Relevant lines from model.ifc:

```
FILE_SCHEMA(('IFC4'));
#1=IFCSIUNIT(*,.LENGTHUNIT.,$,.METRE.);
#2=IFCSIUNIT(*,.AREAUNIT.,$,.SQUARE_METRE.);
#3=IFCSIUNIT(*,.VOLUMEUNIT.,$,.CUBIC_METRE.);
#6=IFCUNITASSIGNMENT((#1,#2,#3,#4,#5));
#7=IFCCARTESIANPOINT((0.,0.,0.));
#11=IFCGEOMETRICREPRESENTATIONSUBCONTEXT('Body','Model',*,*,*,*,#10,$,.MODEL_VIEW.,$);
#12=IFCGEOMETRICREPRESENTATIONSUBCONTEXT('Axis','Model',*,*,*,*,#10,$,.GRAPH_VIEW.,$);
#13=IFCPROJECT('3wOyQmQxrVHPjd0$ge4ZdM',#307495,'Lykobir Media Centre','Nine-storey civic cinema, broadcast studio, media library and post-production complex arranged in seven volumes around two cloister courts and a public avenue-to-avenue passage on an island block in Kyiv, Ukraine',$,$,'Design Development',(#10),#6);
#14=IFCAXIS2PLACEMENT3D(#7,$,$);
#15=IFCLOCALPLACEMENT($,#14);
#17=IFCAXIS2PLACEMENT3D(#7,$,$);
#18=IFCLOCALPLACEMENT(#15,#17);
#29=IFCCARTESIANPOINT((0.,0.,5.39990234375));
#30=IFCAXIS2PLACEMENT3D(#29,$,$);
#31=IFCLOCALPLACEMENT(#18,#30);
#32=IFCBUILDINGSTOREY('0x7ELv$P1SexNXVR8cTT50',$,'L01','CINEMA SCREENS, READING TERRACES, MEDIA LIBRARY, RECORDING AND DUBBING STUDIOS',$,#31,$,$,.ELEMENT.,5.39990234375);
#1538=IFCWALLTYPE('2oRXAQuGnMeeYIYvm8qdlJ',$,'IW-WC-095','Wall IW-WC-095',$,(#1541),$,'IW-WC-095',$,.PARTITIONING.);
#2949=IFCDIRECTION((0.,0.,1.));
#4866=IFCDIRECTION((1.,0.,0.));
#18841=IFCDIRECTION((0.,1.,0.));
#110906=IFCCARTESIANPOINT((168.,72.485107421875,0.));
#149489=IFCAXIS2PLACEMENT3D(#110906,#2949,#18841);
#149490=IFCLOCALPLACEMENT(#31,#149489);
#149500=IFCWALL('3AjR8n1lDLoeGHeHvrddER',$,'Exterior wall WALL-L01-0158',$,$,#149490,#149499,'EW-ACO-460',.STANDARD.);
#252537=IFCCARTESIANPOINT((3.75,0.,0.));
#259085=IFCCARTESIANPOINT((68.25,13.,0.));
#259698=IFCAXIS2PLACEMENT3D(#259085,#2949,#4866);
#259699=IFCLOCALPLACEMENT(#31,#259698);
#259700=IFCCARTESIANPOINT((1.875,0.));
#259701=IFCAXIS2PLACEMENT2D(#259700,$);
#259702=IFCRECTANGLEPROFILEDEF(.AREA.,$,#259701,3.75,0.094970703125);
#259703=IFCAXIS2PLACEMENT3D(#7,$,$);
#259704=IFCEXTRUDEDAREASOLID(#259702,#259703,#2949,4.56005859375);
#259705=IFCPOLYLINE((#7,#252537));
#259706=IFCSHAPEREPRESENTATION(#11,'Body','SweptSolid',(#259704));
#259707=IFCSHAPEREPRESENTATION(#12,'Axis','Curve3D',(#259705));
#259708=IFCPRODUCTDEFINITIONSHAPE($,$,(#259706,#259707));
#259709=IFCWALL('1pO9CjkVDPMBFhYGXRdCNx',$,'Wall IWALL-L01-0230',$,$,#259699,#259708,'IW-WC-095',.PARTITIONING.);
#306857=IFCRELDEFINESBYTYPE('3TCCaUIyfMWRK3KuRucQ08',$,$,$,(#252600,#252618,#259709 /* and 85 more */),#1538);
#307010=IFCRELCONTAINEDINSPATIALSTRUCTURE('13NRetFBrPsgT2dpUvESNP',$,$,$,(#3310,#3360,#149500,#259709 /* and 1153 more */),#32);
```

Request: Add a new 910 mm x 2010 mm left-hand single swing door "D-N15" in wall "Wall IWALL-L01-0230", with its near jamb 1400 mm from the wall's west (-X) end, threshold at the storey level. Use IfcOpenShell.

```python
import numpy as np
import ifcopenshell
import ifcopenshell.api.feature
import ifcopenshell.api.geometry
import ifcopenshell.api.root
import ifcopenshell.api.spatial
import ifcopenshell.geom
import ifcopenshell.util.element
import ifcopenshell.util.placement
import ifcopenshell.util.representation
import ifcopenshell.util.shape
import ifcopenshell.util.unit

model = ifcopenshell.open("model.ifc")
unit_scale = ifcopenshell.util.unit.calculate_unit_scale(model)
settings = ifcopenshell.geom.settings()


def volume(element):
    """Net volume in cubic metres, openings subtracted."""
    shape = ifcopenshell.geom.create_shape(settings, element)
    return ifcopenshell.util.shape.get_volume(shape.geometry)


wall = model.by_guid("1pO9CjkVDPMBFhYGXRdCNx")
storey = ifcopenshell.util.element.get_container(wall, ifc_class="IfcBuildingStorey")
context = ifcopenshell.util.representation.get_context(model, "Model", "Body", "MODEL_VIEW")
before = volume(wall)

width, height, from_end, sill = 0.91, 2.01, 1.4, 0.0  # metres

# The wall runs along its own X axis, and the end named is its -X end.
wall_shape = ifcopenshell.geom.create_shape(settings, wall)
x, y, z = ifcopenshell.util.shape.get_vertices(wall_shape.geometry).T
start = x.min() + from_end
face, thickness = float(y.min()), float(y.max() - y.min())
wall_matrix = ifcopenshell.util.placement.get_local_placement(wall.ObjectPlacement)
level = ifcopenshell.util.placement.get_local_placement(storey.ObjectPlacement)[2, 3]


def in_wall(x, y):
    """Placement at x, y metres in the wall's axes, at sill height."""
    matrix = wall_matrix.copy()
    matrix[:, 3] = wall_matrix @ np.array([x / unit_scale, y / unit_scale, 0.0, 1.0])
    matrix[2, 3] = level + sill / unit_scale
    return matrix


# Opening: a box that overshoots both wall faces by 50 mm.
opening = ifcopenshell.api.root.create_entity(model, ifc_class="IfcOpeningElement", predefined_type="OPENING")
box = ifcopenshell.api.geometry.add_wall_representation(
    model, context=context, length=width, height=height, thickness=thickness + 0.1
)
ifcopenshell.api.geometry.assign_representation(model, product=opening, representation=box)
ifcopenshell.api.geometry.edit_object_placement(model, product=opening, matrix=in_wall(start, face - 0.05), is_si=False)
ifcopenshell.api.feature.add_feature(model, feature=opening, element=wall)

door = ifcopenshell.api.root.create_entity(model, ifc_class="IfcDoor", name="D-N15", predefined_type="DOOR")
door.OverallWidth, door.OverallHeight = width / unit_scale, height / unit_scale
door.OperationType = "SINGLE_SWING_LEFT"
body = ifcopenshell.api.geometry.add_door_representation(
    model,
    context=context,
    overall_width=door.OverallWidth,
    overall_height=door.OverallHeight,
    operation_type="SINGLE_SWING_LEFT",
    lining_properties={"LiningDepth": thickness / unit_scale, "ThresholdDepth": thickness / unit_scale},
)
ifcopenshell.api.geometry.assign_representation(model, product=door, representation=body)
ifcopenshell.api.spatial.assign_container(model, products=[door], relating_structure=storey)
ifcopenshell.api.feature.add_filling(model, opening=opening, element=door)

# The lining spans the wall, so the door starts at the wall face.
ifcopenshell.api.geometry.edit_object_placement(model, product=door, matrix=in_wall(start, face), is_si=False)

after = volume(wall)

print(f"wall volume {before:.3f} -> {after:.3f} m3")

model.write("model-out.ifc")
```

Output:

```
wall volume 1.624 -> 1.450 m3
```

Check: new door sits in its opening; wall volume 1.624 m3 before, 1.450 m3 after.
